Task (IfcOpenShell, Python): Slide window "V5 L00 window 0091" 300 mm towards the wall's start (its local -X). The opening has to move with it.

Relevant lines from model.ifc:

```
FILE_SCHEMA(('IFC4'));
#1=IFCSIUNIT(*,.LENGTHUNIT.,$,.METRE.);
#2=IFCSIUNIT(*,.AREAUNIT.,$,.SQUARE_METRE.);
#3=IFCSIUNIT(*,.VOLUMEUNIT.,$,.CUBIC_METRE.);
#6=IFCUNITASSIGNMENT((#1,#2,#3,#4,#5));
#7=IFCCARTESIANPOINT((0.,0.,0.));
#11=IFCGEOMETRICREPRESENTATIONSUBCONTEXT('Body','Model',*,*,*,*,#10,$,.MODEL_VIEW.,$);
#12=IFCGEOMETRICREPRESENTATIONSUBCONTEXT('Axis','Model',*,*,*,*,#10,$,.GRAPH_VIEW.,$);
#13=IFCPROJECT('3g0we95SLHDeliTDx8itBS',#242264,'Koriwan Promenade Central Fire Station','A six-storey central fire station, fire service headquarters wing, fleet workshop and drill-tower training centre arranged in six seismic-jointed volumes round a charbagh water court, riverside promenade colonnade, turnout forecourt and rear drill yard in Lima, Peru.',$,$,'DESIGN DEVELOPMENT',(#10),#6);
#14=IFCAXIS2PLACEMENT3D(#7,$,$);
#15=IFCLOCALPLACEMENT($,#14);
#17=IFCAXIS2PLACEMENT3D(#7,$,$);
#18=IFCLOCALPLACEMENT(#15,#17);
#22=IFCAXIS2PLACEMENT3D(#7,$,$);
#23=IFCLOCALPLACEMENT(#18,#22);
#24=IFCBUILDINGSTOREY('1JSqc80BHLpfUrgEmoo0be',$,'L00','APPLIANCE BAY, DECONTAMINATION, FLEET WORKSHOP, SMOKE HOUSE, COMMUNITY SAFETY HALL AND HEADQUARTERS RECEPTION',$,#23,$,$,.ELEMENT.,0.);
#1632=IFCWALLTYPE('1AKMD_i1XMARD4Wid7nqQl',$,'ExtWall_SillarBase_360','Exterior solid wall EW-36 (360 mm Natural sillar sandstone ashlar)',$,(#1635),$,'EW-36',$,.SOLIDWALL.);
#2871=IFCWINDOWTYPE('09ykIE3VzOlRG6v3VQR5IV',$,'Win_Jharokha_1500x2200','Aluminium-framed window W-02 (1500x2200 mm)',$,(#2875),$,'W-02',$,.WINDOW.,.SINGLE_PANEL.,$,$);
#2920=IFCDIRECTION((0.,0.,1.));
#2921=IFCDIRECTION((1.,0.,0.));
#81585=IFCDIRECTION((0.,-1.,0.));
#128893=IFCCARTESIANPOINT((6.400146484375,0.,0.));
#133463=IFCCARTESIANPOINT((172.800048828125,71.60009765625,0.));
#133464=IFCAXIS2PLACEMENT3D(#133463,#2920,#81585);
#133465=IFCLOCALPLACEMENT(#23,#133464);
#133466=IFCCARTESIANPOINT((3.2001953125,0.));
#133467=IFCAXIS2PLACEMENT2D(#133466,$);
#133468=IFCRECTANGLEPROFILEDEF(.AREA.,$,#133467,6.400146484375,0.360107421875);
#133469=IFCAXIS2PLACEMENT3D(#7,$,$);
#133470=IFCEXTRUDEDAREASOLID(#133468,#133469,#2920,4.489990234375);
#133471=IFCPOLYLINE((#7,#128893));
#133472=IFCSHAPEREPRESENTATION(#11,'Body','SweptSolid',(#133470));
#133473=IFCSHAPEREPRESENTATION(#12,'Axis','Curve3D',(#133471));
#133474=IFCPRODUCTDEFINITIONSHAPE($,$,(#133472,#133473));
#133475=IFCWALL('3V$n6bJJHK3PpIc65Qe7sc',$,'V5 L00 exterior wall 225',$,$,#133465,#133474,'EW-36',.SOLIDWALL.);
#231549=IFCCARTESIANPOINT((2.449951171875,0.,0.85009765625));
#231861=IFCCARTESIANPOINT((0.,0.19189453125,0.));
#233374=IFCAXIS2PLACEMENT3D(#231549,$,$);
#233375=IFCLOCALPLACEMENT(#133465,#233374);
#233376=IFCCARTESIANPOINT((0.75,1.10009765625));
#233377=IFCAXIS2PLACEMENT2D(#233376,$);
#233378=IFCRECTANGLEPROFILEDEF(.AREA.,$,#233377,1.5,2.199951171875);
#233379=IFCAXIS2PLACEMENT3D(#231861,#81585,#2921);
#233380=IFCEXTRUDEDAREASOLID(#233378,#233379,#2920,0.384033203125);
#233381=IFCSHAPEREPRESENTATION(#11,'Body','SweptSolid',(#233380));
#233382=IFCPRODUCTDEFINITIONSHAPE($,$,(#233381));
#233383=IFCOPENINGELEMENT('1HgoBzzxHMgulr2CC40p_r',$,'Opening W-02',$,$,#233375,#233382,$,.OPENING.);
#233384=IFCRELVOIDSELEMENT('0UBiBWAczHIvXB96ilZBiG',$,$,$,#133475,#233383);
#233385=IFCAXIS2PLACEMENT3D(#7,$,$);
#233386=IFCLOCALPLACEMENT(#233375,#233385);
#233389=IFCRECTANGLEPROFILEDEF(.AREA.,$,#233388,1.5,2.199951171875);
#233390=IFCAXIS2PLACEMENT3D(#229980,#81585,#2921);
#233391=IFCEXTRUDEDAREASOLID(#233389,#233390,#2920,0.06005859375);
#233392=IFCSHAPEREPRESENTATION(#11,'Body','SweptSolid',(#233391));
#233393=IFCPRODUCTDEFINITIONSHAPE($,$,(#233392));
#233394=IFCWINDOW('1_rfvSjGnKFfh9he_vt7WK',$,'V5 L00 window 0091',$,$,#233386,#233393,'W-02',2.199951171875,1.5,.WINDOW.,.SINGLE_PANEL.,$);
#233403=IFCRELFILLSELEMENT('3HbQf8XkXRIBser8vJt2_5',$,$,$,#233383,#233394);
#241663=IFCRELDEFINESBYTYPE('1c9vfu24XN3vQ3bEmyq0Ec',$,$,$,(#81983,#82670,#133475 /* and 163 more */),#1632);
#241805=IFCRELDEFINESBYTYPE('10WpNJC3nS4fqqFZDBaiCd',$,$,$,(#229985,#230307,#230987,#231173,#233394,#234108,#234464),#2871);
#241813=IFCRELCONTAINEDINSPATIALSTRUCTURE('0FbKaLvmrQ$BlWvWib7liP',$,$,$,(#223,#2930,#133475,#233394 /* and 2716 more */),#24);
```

```python
import ifcopenshell
import ifcopenshell.api.geometry
import ifcopenshell.util.placement

model = ifcopenshell.open("model.ifc")

window = model.by_guid("1_rfvSjGnKFfh9he_vt7WK")
opening = window.FillsVoids[0].RelatingOpeningElement
wall = opening.VoidsElements[0].RelatingBuildingElement

wall_matrix = ifcopenshell.util.placement.get_local_placement(wall.ObjectPlacement)
shift = wall_matrix[:3, 0] * -0.3
before = ifcopenshell.util.placement.get_local_placement(window.ObjectPlacement)[:3, 3].copy()

# The window is placed relative to its opening, so it follows when the opening moves.
matrix = ifcopenshell.util.placement.get_local_placement(opening.ObjectPlacement)
matrix[:3, 3] += shift
ifcopenshell.api.geometry.edit_object_placement(
    model, product=opening, matrix=matrix, is_si=False, should_transform_children=True
)

after = ifcopenshell.util.placement.get_local_placement(window.ObjectPlacement)[:3, 3]
print("window moved by", (after - before).round(3) + 0.0)

model.write("model-out.ifc")
```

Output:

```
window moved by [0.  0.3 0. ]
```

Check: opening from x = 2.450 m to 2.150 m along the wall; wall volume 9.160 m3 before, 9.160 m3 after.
